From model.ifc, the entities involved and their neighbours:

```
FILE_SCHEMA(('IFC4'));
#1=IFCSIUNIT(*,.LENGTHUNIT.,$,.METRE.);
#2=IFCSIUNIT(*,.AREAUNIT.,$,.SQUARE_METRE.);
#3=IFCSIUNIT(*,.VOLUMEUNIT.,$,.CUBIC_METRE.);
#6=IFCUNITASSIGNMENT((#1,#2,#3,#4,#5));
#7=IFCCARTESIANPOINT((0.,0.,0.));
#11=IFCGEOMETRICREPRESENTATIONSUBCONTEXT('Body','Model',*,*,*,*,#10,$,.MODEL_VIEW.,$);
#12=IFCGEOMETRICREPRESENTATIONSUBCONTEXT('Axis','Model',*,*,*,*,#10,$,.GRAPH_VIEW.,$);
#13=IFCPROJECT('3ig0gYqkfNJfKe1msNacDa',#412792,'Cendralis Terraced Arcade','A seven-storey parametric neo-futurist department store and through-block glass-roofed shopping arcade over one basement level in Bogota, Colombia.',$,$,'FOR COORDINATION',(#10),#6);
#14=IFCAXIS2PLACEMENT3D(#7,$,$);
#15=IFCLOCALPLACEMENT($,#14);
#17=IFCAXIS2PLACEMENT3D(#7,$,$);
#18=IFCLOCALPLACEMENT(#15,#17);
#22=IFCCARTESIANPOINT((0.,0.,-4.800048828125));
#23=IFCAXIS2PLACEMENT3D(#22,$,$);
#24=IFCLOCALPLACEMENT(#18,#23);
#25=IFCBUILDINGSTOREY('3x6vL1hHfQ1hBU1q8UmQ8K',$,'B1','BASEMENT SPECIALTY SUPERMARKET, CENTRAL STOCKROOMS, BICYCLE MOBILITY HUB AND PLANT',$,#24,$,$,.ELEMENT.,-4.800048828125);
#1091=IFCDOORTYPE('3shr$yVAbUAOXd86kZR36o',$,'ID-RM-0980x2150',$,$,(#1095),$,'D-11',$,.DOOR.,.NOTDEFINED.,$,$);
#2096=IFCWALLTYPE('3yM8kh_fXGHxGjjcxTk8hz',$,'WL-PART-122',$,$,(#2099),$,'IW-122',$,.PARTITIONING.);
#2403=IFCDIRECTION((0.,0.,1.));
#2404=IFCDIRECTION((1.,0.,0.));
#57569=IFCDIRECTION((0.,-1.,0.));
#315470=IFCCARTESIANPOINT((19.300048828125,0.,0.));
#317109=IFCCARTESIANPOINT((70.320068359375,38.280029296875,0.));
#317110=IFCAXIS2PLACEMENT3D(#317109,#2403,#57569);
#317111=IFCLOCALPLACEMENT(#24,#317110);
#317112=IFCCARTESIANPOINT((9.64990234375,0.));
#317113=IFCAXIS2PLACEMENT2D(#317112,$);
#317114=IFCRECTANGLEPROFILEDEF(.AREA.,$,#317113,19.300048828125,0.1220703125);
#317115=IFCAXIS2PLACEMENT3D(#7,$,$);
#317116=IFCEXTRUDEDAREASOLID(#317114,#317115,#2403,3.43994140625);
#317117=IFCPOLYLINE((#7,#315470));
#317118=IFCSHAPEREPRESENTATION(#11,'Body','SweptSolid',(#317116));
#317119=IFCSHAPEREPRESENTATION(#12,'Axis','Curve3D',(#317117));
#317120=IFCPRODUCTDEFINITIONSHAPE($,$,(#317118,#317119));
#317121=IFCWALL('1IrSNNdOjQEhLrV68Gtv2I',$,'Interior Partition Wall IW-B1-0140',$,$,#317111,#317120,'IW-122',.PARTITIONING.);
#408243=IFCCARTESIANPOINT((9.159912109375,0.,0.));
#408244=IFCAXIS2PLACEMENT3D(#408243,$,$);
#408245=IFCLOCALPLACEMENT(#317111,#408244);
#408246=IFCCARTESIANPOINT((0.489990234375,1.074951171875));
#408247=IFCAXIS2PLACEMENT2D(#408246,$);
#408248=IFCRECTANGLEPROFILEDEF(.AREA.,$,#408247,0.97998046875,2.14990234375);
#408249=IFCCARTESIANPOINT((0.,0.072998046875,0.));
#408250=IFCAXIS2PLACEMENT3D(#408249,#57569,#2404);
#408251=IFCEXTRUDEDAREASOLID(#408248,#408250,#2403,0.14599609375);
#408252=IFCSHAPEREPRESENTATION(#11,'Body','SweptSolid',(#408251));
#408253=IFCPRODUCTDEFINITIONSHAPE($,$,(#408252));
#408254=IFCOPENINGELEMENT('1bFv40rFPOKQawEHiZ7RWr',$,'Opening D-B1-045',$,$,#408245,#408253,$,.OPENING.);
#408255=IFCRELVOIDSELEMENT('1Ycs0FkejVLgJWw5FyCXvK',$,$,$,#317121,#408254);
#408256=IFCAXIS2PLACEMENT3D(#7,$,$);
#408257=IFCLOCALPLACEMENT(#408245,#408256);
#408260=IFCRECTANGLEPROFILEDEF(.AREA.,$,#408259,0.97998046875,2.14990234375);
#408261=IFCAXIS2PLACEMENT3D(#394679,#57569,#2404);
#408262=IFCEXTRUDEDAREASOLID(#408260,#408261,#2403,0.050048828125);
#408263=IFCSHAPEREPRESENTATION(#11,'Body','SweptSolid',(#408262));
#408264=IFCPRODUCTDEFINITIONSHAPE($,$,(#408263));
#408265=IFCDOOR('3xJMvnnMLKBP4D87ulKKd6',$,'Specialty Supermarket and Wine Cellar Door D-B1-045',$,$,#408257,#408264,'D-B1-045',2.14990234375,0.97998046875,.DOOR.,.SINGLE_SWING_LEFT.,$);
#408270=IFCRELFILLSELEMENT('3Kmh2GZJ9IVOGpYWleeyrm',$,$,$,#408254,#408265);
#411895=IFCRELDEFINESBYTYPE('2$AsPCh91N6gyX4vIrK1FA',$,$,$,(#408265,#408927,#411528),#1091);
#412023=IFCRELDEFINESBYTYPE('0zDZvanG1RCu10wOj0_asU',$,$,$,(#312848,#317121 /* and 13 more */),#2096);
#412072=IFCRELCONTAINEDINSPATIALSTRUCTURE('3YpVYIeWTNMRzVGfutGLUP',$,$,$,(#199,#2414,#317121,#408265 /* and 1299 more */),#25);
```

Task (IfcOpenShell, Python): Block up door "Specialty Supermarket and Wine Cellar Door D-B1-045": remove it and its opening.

```python
import ifcopenshell
import ifcopenshell.api.feature
import ifcopenshell.api.root
import ifcopenshell.geom
import ifcopenshell.util.shape

model = ifcopenshell.open("model.ifc")
settings = ifcopenshell.geom.settings()


def volume(element):
    """Net volume in cubic metres, openings subtracted."""
    shape = ifcopenshell.geom.create_shape(settings, element)
    return ifcopenshell.util.shape.get_volume(shape.geometry)


door = model.by_guid("3xJMvnnMLKBP4D87ulKKd6")
opening = door.FillsVoids[0].RelatingOpeningElement
wall = opening.VoidsElements[0].RelatingBuildingElement
before = volume(wall)

ifcopenshell.api.root.remove_product(model, product=door)
ifcopenshell.api.feature.remove_feature(model, feature=opening)

after = volume(wall)

print(f"wall volume {before:.3f} -> {after:.3f} m3")

model.write("model_updated.ifc")
```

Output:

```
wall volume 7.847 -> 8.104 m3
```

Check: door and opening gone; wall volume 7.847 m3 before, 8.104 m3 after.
